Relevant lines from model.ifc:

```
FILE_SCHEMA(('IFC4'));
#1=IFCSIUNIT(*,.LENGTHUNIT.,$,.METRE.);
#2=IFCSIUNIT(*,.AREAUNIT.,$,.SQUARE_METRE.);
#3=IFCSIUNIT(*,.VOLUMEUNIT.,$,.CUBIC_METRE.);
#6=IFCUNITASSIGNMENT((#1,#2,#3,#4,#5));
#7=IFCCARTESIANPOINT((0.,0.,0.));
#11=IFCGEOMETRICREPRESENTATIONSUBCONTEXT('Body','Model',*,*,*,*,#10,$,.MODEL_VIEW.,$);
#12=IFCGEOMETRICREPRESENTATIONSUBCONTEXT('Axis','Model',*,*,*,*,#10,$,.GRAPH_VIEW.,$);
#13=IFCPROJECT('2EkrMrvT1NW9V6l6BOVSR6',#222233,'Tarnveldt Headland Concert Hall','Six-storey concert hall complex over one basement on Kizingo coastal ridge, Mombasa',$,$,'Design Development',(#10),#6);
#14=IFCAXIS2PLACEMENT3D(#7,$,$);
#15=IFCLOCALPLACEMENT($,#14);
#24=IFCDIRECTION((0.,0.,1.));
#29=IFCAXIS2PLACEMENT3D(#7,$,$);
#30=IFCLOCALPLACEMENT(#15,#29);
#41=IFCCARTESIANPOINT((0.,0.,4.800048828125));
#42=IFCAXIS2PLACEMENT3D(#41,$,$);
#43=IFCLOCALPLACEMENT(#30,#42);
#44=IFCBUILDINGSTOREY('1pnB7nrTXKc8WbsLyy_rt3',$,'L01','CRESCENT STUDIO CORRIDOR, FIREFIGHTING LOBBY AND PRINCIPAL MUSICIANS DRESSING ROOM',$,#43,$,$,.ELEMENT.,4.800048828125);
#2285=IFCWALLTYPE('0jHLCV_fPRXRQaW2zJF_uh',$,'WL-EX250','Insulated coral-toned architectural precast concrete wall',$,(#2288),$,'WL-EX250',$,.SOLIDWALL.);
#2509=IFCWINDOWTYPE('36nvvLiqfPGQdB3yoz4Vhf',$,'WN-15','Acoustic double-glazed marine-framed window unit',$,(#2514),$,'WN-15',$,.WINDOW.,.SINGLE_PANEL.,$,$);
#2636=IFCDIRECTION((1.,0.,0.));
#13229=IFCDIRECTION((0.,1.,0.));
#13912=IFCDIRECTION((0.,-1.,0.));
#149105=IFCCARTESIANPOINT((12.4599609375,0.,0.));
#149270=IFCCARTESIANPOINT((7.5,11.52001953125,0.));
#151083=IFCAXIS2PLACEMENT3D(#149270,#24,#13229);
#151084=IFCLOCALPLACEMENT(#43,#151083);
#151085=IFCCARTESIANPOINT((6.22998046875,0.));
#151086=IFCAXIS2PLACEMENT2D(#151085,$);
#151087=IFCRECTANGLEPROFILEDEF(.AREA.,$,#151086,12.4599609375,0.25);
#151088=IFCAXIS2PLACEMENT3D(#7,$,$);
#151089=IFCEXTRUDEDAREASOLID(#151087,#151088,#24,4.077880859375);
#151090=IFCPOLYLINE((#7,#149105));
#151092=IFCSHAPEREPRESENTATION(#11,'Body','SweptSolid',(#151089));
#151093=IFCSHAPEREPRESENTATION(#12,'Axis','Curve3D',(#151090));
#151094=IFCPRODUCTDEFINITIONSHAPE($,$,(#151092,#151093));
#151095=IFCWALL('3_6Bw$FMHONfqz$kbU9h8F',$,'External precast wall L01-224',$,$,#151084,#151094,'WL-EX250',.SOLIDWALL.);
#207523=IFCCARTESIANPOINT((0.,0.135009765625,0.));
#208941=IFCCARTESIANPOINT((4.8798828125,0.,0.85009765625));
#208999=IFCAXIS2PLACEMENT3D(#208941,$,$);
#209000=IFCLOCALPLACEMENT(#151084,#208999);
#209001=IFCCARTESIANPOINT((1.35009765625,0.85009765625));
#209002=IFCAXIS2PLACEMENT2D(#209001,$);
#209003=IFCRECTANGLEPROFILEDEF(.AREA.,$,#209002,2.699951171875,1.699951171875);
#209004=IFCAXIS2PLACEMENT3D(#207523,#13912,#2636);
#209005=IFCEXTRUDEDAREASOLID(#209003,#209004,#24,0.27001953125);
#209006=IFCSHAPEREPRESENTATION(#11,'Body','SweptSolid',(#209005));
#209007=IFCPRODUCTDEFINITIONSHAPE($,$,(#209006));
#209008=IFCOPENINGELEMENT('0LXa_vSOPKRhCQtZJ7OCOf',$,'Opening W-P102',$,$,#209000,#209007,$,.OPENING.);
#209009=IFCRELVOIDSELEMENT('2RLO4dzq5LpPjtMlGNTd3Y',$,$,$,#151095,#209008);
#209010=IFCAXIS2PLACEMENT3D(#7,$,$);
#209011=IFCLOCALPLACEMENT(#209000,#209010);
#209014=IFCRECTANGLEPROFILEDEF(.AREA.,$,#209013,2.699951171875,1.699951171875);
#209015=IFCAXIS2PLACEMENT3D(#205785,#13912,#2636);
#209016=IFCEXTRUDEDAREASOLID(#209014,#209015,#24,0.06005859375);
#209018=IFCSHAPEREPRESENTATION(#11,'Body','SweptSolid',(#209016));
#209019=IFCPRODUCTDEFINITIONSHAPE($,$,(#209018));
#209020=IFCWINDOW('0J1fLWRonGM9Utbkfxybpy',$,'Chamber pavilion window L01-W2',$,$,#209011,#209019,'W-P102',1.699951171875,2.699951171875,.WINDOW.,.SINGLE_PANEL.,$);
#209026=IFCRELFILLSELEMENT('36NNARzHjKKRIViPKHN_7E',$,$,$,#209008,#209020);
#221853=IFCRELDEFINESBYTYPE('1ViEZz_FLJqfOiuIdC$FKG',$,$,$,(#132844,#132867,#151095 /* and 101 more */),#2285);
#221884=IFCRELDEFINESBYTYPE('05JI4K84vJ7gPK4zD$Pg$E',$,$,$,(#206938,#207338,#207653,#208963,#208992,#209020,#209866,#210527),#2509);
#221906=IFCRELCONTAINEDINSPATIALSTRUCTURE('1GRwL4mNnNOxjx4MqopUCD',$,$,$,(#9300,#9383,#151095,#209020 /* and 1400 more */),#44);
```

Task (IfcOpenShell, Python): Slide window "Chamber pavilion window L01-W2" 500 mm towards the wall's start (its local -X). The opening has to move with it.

```python
import ifcopenshell
import ifcopenshell.api.geometry
import ifcopenshell.util.placement

model = ifcopenshell.open("model.ifc")

window = model.by_guid("0J1fLWRonGM9Utbkfxybpy")
opening = window.FillsVoids[0].RelatingOpeningElement
wall = opening.VoidsElements[0].RelatingBuildingElement

wall_matrix = ifcopenshell.util.placement.get_local_placement(wall.ObjectPlacement)
shift = wall_matrix[:3, 0] * -0.5
before = ifcopenshell.util.placement.get_local_placement(window.ObjectPlacement)[:3, 3].copy()

# The window is placed relative to its opening, so it follows when the opening moves.
matrix = ifcopenshell.util.placement.get_local_placement(opening.ObjectPlacement)
matrix[:3, 3] += shift
ifcopenshell.api.geometry.edit_object_placement(
    model, product=opening, matrix=matrix, is_si=False, should_transform_children=True
)

after = ifcopenshell.util.placement.get_local_placement(window.ObjectPlacement)[:3, 3]
print("window moved by", (after - before).round(3) + 0.0)

model.write("model-out.ifc")
```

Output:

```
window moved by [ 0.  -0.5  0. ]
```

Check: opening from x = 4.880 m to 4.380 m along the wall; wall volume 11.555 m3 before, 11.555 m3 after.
